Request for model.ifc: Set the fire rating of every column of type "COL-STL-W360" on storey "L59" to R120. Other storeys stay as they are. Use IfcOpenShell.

First a look at what the model holds.

```python
import ifcopenshell
import ifcopenshell.util.element

model = ifcopenshell.open("model.ifc")
print(model.schema)
storey = next(s for s in model.by_type("IfcBuildingStorey") if s.Name == "L59")
columns = [e for e in ifcopenshell.util.element.get_decomposition(storey) if e.is_a("IfcColumn")]
seen = {}
for e in columns:
    element_type = ifcopenshell.util.element.get_type(e)
    key = (element_type.Name if element_type != e and element_type else None, ifcopenshell.util.element.get_pset(e, "Pset_ColumnCommon", "FireRating"))
    seen[key] = seen.get(key, 0) + 1
for (name, value), count in sorted(seen.items(), key=str):
    print(count, "x", name, "|", value)
```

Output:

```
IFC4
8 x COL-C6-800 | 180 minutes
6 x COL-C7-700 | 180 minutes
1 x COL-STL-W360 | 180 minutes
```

```python
import ifcopenshell
import ifcopenshell.api.pset
import ifcopenshell.util.element

model = ifcopenshell.open("model.ifc")

storey = next(s for s in model.by_type("IfcBuildingStorey") if s.Name == "L59")
columns = [e for e in ifcopenshell.util.element.get_decomposition(storey) if e.is_a("IfcColumn")]

count = 0
for e in columns:
    element_type = ifcopenshell.util.element.get_type(e)
    if element_type in (None, e) or element_type.Name != "COL-STL-W360":
        continue
    found = ifcopenshell.util.element.get_pset(e, "Pset_ColumnCommon", should_inherit=False)
    if found:
        pset = model.by_id(found["id"])
        if len(ifcopenshell.util.element.get_elements_by_pset(pset)) > 1:
            pset = ifcopenshell.api.pset.unshare_pset(model, products=[e], pset=pset)[0]
    else:
        pset = ifcopenshell.api.pset.add_pset(model, product=e, name="Pset_ColumnCommon")
    ifcopenshell.api.pset.edit_pset(model, pset=pset, properties={"FireRating": "R120"})
    count += 1

print(count, "columns updated")

model.write("model-out.ifc")
```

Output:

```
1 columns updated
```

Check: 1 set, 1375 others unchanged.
